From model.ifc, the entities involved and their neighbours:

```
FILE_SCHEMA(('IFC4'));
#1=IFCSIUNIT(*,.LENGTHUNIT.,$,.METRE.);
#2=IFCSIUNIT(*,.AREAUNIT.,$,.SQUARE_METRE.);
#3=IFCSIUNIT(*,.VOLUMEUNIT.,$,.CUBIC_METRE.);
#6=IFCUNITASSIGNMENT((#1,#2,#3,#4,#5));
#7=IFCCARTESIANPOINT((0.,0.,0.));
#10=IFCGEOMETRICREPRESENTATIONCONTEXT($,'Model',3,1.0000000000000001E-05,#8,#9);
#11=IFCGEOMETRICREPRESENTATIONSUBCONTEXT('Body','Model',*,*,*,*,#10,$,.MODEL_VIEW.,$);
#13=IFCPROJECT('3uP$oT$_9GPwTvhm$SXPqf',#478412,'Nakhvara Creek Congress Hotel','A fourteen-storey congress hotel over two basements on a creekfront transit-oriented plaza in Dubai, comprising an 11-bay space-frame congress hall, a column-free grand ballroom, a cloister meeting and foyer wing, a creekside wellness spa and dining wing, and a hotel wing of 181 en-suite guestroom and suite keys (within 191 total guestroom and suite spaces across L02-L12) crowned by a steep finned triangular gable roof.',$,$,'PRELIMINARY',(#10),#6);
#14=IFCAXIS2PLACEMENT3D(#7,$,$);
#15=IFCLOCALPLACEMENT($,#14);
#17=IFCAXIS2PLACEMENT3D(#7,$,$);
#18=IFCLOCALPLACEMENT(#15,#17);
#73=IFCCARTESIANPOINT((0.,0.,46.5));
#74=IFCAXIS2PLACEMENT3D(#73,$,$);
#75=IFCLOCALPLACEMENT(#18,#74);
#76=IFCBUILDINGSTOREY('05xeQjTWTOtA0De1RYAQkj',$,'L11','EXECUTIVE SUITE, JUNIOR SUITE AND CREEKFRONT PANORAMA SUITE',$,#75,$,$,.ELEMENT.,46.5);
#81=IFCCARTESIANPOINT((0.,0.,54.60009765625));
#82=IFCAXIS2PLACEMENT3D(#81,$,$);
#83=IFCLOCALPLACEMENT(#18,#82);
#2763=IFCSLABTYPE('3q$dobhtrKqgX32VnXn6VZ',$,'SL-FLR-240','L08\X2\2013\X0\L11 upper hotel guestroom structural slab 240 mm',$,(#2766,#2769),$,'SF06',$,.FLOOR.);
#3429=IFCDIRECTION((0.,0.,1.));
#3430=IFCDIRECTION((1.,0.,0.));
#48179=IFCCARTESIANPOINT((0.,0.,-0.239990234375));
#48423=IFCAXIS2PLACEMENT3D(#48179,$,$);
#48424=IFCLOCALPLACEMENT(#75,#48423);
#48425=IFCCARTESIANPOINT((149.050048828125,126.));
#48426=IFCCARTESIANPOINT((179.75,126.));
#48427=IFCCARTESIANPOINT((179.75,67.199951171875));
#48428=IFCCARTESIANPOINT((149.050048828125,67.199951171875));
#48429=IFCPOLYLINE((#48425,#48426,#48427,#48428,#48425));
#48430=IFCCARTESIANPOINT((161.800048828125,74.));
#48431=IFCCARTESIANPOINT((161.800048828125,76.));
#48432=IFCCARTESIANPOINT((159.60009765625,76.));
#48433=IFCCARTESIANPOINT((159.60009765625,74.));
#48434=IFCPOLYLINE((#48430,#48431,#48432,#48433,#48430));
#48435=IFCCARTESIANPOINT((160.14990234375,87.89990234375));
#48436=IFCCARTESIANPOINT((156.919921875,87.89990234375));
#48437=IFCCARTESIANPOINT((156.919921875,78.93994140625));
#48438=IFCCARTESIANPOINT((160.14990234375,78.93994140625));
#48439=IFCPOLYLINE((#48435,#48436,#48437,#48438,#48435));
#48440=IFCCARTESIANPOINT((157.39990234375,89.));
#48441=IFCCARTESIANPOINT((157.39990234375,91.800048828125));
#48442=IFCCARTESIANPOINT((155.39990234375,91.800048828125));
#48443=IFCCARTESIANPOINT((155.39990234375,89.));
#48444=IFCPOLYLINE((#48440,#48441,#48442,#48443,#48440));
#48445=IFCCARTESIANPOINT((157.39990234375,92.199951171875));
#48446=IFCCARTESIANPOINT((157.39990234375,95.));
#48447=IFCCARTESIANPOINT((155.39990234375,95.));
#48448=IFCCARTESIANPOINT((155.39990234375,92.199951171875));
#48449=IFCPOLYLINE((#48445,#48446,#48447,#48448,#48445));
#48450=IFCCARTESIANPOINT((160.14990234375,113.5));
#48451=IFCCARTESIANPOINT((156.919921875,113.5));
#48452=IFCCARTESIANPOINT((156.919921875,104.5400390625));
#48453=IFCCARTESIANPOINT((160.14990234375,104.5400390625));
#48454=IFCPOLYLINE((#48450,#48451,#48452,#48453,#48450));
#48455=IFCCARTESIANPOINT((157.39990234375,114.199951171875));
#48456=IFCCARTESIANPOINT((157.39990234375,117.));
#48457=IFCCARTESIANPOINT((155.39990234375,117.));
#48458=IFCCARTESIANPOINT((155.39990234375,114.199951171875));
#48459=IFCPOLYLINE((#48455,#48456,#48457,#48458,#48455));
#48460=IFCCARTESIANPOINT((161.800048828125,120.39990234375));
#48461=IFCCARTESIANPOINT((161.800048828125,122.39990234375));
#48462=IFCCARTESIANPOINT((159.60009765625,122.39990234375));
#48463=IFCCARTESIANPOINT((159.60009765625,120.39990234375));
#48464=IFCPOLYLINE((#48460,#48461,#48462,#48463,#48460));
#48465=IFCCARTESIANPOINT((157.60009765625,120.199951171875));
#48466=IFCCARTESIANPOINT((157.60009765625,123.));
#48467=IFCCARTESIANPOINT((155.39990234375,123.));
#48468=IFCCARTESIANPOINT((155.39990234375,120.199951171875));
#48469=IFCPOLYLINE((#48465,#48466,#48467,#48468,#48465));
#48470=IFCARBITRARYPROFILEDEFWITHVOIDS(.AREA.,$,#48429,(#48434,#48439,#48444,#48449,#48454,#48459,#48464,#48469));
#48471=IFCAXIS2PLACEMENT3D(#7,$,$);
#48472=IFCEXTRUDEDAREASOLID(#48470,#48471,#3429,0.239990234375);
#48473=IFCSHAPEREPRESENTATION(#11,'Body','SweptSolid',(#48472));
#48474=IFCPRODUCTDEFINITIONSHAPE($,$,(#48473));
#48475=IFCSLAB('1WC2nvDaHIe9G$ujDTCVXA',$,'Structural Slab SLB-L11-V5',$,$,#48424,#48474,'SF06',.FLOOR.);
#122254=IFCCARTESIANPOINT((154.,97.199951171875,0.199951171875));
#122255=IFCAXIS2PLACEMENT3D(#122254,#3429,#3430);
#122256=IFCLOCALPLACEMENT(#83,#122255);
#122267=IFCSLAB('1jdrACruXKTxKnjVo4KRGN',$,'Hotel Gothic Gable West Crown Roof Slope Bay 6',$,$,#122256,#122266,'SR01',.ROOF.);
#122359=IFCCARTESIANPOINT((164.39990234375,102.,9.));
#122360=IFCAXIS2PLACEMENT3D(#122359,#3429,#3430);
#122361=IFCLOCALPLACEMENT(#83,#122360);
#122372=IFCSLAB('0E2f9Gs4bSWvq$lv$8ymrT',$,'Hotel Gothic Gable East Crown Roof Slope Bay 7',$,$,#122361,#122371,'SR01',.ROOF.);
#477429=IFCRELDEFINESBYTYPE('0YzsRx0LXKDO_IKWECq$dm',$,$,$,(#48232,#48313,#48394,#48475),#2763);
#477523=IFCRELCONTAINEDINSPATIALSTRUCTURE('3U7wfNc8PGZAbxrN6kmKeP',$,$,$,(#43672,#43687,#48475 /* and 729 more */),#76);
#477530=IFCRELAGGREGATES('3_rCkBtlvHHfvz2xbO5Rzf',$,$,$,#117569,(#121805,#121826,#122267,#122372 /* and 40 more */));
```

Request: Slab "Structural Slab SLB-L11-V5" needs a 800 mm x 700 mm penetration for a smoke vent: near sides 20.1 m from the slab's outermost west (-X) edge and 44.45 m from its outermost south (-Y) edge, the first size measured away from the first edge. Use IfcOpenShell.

```python
import numpy as np
import ifcopenshell
import ifcopenshell.api.feature
import ifcopenshell.api.geometry
import ifcopenshell.api.root
import ifcopenshell.geom
import ifcopenshell.util.placement
import ifcopenshell.util.representation
import ifcopenshell.util.shape
import ifcopenshell.util.unit

model = ifcopenshell.open("model.ifc")
unit_scale = ifcopenshell.util.unit.calculate_unit_scale(model)
settings = ifcopenshell.geom.settings()


def volume(element):
    """Net volume in cubic metres, openings subtracted."""
    shape = ifcopenshell.geom.create_shape(settings, element)
    return ifcopenshell.util.shape.get_volume(shape.geometry)


slab = model.by_guid("1WC2nvDaHIe9G$ujDTCVXA")
before = volume(slab)

# Extent in the slab's own axes, in metres. The edges named are its -X and -Y sides.
slab_shape = ifcopenshell.geom.create_shape(settings, slab)
vertices = ifcopenshell.util.shape.get_vertices(slab_shape.geometry)
x_min, y_min, bottom = vertices.min(axis=0)
top = vertices[:, 2].max()

opening = ifcopenshell.api.root.create_entity(model, ifc_class="IfcOpeningElement", name="Smoke vent opening", predefined_type="OPENING")
context = ifcopenshell.util.representation.get_context(model, "Model", "Body", "MODEL_VIEW")
width, depth = 0.8, 0.7
outline = [(0.0, 0.0), (width, 0.0), (width, depth), (0.0, depth), (0.0, 0.0)]
# Overshoot both faces by 50 mm so the cut is clean.
shape = ifcopenshell.api.geometry.add_slab_representation(
    model, context=context, depth=top - bottom + 0.1, polyline=outline
)
ifcopenshell.api.geometry.assign_representation(model, product=opening, representation=shape)

matrix = ifcopenshell.util.placement.get_local_placement(slab.ObjectPlacement)
matrix[:, 3] = matrix @ np.append(np.array([x_min + 20.1, y_min + 44.45, bottom - 0.05]) / unit_scale, 1.0)
ifcopenshell.api.geometry.edit_object_placement(model, product=opening, matrix=matrix, is_si=False)
ifcopenshell.api.feature.add_feature(model, feature=opening, element=slab)

after = volume(slab)

print(f"slab volume {before:.3f} -> {after:.3f} m3")

model.write("model-out.ifc")
```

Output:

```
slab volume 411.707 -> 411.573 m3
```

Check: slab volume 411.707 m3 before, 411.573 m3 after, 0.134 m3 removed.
